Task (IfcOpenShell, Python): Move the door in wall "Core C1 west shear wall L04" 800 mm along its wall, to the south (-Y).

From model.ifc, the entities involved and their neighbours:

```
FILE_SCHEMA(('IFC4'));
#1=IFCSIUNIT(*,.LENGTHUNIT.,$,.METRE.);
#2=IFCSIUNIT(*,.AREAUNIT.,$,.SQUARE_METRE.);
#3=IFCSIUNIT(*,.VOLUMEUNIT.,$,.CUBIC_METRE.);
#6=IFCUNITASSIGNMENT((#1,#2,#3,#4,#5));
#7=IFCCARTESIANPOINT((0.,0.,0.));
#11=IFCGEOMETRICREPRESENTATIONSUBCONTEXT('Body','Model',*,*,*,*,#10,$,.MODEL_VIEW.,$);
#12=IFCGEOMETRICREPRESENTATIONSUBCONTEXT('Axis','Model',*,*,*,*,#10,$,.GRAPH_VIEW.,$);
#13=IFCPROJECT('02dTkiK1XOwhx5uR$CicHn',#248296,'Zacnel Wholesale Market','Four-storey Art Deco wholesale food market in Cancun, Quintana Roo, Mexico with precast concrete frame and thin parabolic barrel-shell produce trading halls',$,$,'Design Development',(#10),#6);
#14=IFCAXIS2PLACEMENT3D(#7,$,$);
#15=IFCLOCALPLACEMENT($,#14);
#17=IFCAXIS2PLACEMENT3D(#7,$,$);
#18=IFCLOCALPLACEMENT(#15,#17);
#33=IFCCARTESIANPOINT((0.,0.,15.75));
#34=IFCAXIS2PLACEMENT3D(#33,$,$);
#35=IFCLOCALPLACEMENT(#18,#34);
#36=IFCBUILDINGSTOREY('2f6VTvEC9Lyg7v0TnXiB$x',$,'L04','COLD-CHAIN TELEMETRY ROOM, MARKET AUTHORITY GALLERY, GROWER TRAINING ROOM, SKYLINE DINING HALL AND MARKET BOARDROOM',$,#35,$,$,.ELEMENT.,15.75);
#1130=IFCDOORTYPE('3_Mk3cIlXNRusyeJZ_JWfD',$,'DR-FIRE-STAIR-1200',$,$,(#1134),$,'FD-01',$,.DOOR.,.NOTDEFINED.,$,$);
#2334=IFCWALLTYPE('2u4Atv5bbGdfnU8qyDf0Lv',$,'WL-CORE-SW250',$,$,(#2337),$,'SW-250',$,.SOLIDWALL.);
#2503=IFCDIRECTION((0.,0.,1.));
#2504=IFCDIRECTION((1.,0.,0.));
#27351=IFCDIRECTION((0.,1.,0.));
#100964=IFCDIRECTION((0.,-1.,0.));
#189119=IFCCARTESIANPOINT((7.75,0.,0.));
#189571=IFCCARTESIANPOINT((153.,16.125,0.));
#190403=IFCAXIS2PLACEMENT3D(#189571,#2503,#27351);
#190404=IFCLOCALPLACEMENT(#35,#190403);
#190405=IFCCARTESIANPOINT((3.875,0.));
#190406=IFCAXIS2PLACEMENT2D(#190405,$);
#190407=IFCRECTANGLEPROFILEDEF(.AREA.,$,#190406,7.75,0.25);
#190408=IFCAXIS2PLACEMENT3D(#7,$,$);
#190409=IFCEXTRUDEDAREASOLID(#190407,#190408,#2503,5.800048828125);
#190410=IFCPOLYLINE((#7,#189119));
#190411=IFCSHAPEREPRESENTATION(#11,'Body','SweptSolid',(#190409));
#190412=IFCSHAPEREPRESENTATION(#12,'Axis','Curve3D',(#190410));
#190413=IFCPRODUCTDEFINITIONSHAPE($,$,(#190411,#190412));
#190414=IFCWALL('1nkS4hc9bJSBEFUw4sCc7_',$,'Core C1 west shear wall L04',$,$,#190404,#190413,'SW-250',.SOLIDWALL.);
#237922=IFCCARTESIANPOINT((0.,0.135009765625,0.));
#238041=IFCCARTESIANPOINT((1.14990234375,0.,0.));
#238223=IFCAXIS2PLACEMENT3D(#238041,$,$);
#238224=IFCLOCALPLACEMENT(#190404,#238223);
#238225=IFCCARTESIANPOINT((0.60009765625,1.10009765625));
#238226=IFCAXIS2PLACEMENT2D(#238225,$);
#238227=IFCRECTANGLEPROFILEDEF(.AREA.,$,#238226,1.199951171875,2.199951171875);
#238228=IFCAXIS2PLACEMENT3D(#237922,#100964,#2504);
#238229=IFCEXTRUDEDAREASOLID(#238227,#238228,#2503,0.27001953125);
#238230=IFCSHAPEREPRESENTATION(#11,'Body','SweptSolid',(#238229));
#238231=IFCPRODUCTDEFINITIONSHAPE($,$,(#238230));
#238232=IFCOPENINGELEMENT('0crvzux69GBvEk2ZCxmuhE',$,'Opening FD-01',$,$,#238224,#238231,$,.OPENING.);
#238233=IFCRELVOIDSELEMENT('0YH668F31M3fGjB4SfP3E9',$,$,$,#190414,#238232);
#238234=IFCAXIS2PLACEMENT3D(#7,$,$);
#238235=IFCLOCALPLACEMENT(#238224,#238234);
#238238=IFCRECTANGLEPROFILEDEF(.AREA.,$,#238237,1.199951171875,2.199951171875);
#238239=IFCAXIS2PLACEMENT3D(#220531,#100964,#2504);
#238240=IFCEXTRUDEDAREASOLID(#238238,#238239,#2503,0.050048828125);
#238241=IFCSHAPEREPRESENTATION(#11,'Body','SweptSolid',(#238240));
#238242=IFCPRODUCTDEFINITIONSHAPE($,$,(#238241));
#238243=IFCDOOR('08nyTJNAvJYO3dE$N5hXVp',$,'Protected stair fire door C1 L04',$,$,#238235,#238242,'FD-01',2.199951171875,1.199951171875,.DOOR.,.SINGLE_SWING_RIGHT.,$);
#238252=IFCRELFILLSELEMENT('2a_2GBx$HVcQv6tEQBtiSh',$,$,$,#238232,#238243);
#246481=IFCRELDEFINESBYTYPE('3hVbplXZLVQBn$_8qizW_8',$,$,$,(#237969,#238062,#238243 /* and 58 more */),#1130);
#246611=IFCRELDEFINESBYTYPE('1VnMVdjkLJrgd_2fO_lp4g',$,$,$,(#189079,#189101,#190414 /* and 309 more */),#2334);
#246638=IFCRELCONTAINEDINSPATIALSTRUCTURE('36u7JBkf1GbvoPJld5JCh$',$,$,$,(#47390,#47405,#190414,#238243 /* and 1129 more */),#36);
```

```python
import ifcopenshell
import ifcopenshell.api.geometry
import ifcopenshell.util.placement
import ifcopenshell.util.unit

model = ifcopenshell.open("model.ifc")
unit_scale = ifcopenshell.util.unit.calculate_unit_scale(model)

door = model.by_guid("08nyTJNAvJYO3dE$N5hXVp")
opening = door.FillsVoids[0].RelatingOpeningElement
wall = opening.VoidsElements[0].RelatingBuildingElement

wall_matrix = ifcopenshell.util.placement.get_local_placement(wall.ObjectPlacement)
shift = wall_matrix[:3, 0] * -0.8 / unit_scale
before = ifcopenshell.util.placement.get_local_placement(door.ObjectPlacement)[:3, 3].copy()

# The door is placed relative to its opening, so it follows when the opening moves.
matrix = ifcopenshell.util.placement.get_local_placement(opening.ObjectPlacement)
matrix[:3, 3] += shift
ifcopenshell.api.geometry.edit_object_placement(
    model, product=opening, matrix=matrix, is_si=False, should_transform_children=True
)

after = ifcopenshell.util.placement.get_local_placement(door.ObjectPlacement)[:3, 3]
print("door moved by", (after - before).round(3) + 0.0)

model.write("model_edited.ifc")
```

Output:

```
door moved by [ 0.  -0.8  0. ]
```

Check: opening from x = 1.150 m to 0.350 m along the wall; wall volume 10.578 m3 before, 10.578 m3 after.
